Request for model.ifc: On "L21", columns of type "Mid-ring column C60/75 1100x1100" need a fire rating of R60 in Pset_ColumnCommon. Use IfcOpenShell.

First a look at what the model holds.

```python
import ifcopenshell
import ifcopenshell.util.element

model = ifcopenshell.open("model.ifc")
print(model.schema)
storey = next(s for s in model.by_type("IfcBuildingStorey") if s.Name == "L21")
columns = [e for e in ifcopenshell.util.element.get_decomposition(storey) if e.is_a("IfcColumn")]
seen = {}
for e in columns:
    element_type = ifcopenshell.util.element.get_type(e)
    key = (element_type.Name if element_type != e and element_type else None, ifcopenshell.util.element.get_pset(e, "Pset_ColumnCommon", "FireRating"))
    seen[key] = seen.get(key, 0) + 1
for (name, value), count in sorted(seen.items(), key=str):
    print(count, "x", name, "|", value)
```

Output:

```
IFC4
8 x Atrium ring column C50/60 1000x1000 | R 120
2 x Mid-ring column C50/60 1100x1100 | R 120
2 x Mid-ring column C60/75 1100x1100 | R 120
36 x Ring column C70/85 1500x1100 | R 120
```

```python
import ifcopenshell
import ifcopenshell.api.pset
import ifcopenshell.util.element

model = ifcopenshell.open("model.ifc")

storey = next(s for s in model.by_type("IfcBuildingStorey") if s.Name == "L21")
columns = [e for e in ifcopenshell.util.element.get_decomposition(storey) if e.is_a("IfcColumn")]

count = 0
for e in columns:
    element_type = ifcopenshell.util.element.get_type(e)
    if element_type in (None, e) or element_type.Name != "Mid-ring column C60/75 1100x1100":
        continue
    found = ifcopenshell.util.element.get_pset(e, "Pset_ColumnCommon", should_inherit=False)
    if found:
        pset = model.by_id(found["id"])
        if len(ifcopenshell.util.element.get_elements_by_pset(pset)) > 1:
            pset = ifcopenshell.api.pset.unshare_pset(model, products=[e], pset=pset)[0]
    else:
        pset = ifcopenshell.api.pset.add_pset(model, product=e, name="Pset_ColumnCommon")
    ifcopenshell.api.pset.edit_pset(model, pset=pset, properties={"FireRating": "R60"})
    count += 1

print(count, "columns updated")

model.write("model_v2.ifc")
```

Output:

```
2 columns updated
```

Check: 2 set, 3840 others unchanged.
